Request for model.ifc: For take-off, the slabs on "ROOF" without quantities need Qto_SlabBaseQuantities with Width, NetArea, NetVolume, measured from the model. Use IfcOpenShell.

First a look at what the model holds.

```python
import ifcopenshell
import ifcopenshell.util.element
import ifcopenshell.util.unit

model = ifcopenshell.open("model.ifc")
print(model.schema)
for unit_type in ("LENGTHUNIT", "AREAUNIT", "VOLUMEUNIT"):
    print(unit_type, ifcopenshell.util.unit.calculate_unit_scale(model, unit_type))
storey = next(s for s in model.by_type("IfcBuildingStorey") if s.Name == "ROOF")
slabs = [e for e in ifcopenshell.util.element.get_decomposition(storey) if e.is_a("IfcSlab")]
for e in sorted(slabs, key=lambda e: e.id()):
    print(e.id(), e.is_a(), e.Name, list(ifcopenshell.util.element.get_psets(e, qtos_only=True)), sep=" | ")
```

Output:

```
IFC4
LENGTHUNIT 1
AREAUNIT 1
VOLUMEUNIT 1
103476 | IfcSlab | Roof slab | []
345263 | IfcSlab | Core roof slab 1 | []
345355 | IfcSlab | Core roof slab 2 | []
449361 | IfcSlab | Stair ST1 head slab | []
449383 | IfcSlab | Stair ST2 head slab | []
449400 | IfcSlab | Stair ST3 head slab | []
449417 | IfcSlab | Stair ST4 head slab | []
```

```python
import ifcopenshell
import ifcopenshell.api.pset
import ifcopenshell.geom
import ifcopenshell.util.element
import ifcopenshell.util.shape
import ifcopenshell.util.unit

model = ifcopenshell.open("model.ifc")
unit_scale = ifcopenshell.util.unit.calculate_unit_scale(model)
area_scale = ifcopenshell.util.unit.calculate_unit_scale(model, "AREAUNIT")
volume_scale = ifcopenshell.util.unit.calculate_unit_scale(model, "VOLUMEUNIT")
settings = ifcopenshell.geom.settings()

storey = next(s for s in model.by_type("IfcBuildingStorey") if s.Name == "ROOF")
slabs = [e for e in ifcopenshell.util.element.get_decomposition(storey) if e.is_a("IfcSlab")]

for e in sorted(slabs, key=lambda e: e.id()):
    if ifcopenshell.util.element.get_psets(e, qtos_only=True, should_inherit=False):
        continue
    # Geometry comes back in metres, in the element's own axes.
    shape = ifcopenshell.geom.create_shape(settings, e)
    values = {
        "Width": ifcopenshell.util.shape.get_z(shape.geometry) / unit_scale,
        "NetArea": ifcopenshell.util.shape.get_footprint_area(shape.geometry) / area_scale,
        "NetVolume": ifcopenshell.util.shape.get_volume(shape.geometry) / volume_scale,
    }
    qto = ifcopenshell.api.pset.add_qto(model, product=e, name="Qto_SlabBaseQuantities")
    ifcopenshell.api.pset.edit_qto(model, qto=qto, properties=values)
    print(e.id(), {k: round(v, 3) for k, v in values.items()})

model.write("model_rev.ifc")
```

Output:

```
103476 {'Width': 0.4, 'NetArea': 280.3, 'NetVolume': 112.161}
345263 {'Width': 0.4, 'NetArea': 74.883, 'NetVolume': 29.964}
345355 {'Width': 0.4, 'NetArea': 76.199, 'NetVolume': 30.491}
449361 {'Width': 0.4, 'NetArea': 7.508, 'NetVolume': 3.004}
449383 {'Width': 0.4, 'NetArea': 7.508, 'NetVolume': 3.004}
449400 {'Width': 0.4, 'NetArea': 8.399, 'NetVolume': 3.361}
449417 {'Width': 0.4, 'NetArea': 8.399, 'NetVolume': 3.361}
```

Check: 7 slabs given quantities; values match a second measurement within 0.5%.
